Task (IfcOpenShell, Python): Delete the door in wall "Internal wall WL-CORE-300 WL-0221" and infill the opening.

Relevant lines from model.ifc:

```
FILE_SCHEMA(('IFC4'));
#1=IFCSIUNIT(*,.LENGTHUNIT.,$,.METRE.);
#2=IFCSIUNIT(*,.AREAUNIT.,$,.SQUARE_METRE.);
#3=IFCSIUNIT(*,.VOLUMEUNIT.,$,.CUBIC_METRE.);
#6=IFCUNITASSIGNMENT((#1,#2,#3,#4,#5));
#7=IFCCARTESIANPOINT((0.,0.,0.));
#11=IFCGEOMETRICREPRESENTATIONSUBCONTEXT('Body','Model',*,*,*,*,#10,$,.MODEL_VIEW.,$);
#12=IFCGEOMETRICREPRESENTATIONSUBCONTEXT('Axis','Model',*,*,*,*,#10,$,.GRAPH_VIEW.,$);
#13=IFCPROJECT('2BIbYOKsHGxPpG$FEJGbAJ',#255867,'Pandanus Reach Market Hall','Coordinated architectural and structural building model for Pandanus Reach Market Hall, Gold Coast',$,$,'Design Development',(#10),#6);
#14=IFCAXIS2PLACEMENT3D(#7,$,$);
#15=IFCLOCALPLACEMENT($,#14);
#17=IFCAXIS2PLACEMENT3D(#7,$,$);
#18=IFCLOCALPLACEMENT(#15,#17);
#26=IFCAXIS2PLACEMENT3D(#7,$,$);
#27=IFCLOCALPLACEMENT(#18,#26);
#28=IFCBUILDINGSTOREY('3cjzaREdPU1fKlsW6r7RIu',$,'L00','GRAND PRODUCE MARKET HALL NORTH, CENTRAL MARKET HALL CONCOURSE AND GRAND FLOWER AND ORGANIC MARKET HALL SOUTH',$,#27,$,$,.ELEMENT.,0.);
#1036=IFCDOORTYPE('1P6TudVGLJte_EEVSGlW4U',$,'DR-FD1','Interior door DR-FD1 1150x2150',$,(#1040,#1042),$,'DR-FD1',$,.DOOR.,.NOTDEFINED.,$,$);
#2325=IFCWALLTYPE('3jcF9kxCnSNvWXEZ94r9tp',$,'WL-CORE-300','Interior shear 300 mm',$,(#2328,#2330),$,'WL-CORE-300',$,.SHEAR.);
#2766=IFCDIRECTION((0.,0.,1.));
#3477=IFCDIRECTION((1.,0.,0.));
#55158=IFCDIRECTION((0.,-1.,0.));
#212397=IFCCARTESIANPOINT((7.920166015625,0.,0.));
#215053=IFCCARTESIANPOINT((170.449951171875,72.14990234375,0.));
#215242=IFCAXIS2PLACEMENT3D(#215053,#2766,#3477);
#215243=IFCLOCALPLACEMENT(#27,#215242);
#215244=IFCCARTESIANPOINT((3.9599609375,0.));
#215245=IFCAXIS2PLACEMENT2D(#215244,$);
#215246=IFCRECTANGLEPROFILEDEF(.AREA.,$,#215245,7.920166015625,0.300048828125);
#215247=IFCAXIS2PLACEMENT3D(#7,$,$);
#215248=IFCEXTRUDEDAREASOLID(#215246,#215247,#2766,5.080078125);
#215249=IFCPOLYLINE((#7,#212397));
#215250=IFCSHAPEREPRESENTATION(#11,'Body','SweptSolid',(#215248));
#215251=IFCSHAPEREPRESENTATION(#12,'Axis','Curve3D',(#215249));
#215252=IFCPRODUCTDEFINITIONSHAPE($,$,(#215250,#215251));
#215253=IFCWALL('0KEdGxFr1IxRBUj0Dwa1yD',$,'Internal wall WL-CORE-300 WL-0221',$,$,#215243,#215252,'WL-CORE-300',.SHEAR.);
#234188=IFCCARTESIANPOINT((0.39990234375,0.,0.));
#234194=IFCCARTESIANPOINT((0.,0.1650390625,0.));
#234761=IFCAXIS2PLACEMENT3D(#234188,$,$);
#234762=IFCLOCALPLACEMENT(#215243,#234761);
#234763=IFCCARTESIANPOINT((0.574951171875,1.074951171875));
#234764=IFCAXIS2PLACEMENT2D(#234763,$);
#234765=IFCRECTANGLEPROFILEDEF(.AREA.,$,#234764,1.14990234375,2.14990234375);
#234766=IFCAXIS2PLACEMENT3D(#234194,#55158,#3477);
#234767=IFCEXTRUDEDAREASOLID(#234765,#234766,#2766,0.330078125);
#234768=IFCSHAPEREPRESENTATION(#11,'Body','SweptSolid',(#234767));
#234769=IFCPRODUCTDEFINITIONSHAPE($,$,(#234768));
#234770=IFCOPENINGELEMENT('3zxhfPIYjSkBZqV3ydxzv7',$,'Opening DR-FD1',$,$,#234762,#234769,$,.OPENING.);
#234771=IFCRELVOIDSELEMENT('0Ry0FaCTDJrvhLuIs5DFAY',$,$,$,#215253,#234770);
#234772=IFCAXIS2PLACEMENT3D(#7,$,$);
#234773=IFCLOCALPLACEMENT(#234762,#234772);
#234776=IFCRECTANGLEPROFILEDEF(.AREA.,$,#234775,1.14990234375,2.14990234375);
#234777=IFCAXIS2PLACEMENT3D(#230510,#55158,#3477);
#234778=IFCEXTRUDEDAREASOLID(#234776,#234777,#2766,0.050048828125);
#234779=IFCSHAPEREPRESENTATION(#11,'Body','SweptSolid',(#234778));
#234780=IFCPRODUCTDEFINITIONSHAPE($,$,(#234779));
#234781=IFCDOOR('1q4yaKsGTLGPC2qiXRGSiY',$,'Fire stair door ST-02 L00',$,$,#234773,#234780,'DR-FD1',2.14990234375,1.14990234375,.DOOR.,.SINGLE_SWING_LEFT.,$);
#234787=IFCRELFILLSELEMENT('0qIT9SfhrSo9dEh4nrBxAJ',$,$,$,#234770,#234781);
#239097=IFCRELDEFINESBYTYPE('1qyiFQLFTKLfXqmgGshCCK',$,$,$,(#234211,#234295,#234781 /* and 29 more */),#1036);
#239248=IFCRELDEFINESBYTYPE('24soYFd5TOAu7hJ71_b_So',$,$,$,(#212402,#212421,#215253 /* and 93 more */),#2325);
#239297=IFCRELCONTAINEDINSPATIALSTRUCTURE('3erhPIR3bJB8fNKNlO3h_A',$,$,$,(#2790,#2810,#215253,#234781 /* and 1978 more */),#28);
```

```python
import ifcopenshell
import ifcopenshell.api.feature
import ifcopenshell.api.root
import ifcopenshell.geom
import ifcopenshell.util.shape

model = ifcopenshell.open("model.ifc")
settings = ifcopenshell.geom.settings()


def volume(element):
    """Net volume in cubic metres, openings subtracted."""
    shape = ifcopenshell.geom.create_shape(settings, element)
    return ifcopenshell.util.shape.get_volume(shape.geometry)


door = model.by_guid("1q4yaKsGTLGPC2qiXRGSiY")
opening = door.FillsVoids[0].RelatingOpeningElement
wall = opening.VoidsElements[0].RelatingBuildingElement
before = volume(wall)

ifcopenshell.api.root.remove_product(model, product=door)
ifcopenshell.api.feature.remove_feature(model, feature=opening)

after = volume(wall)

print(f"wall volume {before:.3f} -> {after:.3f} m3")

model.write("model_edited.ifc")
```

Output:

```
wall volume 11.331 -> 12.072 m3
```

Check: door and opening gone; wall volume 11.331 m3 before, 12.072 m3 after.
